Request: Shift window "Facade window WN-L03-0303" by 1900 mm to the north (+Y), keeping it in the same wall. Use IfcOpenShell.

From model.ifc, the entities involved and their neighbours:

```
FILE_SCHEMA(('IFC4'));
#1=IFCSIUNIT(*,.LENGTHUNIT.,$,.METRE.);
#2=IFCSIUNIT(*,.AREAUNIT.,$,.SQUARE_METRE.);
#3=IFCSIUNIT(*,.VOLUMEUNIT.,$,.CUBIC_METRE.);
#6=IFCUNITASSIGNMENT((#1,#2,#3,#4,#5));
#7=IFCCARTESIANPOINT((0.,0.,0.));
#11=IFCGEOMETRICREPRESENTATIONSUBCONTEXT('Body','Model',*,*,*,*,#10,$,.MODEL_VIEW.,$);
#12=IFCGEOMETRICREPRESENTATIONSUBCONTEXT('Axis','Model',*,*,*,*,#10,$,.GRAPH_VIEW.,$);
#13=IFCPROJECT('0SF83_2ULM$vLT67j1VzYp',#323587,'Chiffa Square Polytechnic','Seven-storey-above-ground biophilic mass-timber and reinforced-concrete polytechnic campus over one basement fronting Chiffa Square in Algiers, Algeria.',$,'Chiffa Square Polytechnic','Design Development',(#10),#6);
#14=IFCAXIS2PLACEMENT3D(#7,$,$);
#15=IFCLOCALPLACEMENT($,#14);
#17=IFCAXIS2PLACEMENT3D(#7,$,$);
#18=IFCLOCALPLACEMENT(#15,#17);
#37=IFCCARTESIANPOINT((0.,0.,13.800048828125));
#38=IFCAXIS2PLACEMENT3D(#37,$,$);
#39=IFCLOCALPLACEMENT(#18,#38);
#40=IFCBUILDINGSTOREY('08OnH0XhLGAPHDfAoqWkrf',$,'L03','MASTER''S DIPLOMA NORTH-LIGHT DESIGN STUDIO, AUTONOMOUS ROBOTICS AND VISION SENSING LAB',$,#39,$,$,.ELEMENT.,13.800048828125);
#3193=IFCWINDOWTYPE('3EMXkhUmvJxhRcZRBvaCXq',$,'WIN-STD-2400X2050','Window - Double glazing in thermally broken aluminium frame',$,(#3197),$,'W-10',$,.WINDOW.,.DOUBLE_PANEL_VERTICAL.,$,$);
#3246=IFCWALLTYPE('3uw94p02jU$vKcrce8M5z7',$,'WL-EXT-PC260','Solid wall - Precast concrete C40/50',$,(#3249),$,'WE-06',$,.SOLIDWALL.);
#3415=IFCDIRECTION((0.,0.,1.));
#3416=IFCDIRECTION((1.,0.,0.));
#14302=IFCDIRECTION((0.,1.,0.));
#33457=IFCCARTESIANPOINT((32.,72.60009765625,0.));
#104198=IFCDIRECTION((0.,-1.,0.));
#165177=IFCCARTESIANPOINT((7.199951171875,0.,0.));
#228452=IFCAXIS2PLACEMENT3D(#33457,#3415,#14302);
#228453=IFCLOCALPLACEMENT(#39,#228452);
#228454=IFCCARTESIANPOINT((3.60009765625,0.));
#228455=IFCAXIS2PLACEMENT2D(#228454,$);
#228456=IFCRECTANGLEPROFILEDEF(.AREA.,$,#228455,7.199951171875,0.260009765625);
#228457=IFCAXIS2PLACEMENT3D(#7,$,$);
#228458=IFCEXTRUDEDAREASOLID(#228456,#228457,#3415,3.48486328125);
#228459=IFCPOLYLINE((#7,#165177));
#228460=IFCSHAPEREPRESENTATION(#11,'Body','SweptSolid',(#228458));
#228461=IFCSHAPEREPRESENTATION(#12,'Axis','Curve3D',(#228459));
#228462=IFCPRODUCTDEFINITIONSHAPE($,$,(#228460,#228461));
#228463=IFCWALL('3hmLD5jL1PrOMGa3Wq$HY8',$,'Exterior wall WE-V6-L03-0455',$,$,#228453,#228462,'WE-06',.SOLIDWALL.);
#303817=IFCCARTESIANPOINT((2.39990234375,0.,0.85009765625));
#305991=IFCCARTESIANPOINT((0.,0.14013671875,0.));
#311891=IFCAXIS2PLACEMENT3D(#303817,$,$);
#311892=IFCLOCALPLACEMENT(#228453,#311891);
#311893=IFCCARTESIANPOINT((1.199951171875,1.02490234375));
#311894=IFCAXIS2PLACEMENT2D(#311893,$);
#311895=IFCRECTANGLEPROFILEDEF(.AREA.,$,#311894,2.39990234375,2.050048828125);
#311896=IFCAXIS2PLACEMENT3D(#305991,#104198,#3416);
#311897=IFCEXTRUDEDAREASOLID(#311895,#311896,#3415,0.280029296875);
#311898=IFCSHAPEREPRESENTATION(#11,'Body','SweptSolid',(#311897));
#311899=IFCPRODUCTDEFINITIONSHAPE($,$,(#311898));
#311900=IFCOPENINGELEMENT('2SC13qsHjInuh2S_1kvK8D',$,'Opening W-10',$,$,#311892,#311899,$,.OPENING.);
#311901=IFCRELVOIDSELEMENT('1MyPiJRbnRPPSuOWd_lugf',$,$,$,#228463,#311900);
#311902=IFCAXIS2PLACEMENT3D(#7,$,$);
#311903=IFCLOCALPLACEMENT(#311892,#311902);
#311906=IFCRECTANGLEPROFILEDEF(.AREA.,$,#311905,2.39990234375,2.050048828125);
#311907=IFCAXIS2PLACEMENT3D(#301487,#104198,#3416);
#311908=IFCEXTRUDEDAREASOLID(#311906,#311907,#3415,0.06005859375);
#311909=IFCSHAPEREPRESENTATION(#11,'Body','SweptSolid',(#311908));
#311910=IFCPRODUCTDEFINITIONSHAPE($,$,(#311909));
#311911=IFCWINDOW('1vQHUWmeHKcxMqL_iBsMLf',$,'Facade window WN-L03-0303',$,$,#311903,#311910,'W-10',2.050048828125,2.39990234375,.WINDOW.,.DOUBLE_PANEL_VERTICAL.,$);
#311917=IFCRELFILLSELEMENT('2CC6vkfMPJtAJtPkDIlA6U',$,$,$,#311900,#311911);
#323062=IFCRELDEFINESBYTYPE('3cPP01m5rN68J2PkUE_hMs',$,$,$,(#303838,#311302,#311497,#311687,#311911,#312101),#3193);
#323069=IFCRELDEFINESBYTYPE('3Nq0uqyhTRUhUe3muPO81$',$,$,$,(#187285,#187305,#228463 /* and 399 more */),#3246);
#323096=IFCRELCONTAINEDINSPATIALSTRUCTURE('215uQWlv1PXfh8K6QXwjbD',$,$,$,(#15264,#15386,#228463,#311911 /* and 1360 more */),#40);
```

```python
import ifcopenshell
import ifcopenshell.api.geometry
import ifcopenshell.util.placement
import ifcopenshell.util.unit

model = ifcopenshell.open("model.ifc")
unit_scale = ifcopenshell.util.unit.calculate_unit_scale(model)

window = model.by_id(311911)
opening = window.FillsVoids[0].RelatingOpeningElement
wall = opening.VoidsElements[0].RelatingBuildingElement

wall_matrix = ifcopenshell.util.placement.get_local_placement(wall.ObjectPlacement)
shift = wall_matrix[:3, 0] * 1.9 / unit_scale
before = ifcopenshell.util.placement.get_local_placement(window.ObjectPlacement)[:3, 3].copy()

# The window is placed relative to its opening, so it follows when the opening moves.
matrix = ifcopenshell.util.placement.get_local_placement(opening.ObjectPlacement)
matrix[:3, 3] += shift
ifcopenshell.api.geometry.edit_object_placement(
    model, product=opening, matrix=matrix, is_si=False, should_transform_children=True
)

after = ifcopenshell.util.placement.get_local_placement(window.ObjectPlacement)[:3, 3]
print("window moved by", (after - before).round(3) + 0.0)

model.write("model_rev.ifc")
```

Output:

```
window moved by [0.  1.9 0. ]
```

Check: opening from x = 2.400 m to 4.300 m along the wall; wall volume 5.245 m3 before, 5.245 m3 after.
